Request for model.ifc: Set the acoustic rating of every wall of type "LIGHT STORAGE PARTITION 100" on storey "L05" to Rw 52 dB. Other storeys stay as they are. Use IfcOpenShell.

First a look at what the model holds.

```python
import ifcopenshell
import ifcopenshell.util.element

model = ifcopenshell.open("model.ifc")
print(model.schema)
storey = next(s for s in model.by_type("IfcBuildingStorey") if s.Name == "L05")
walls = [e for e in ifcopenshell.util.element.get_decomposition(storey) if e.is_a("IfcWall")]
seen = {}
for e in walls:
    element_type = ifcopenshell.util.element.get_type(e)
    key = (element_type.Name if element_type != e and element_type else None, ifcopenshell.util.element.get_pset(e, "Pset_WallCommon", "AcousticRating"))
    seen[key] = seen.get(key, 0) + 1
for (name, value), count in sorted(seen.items(), key=str):
    print(count, "x", name, "|", value)
```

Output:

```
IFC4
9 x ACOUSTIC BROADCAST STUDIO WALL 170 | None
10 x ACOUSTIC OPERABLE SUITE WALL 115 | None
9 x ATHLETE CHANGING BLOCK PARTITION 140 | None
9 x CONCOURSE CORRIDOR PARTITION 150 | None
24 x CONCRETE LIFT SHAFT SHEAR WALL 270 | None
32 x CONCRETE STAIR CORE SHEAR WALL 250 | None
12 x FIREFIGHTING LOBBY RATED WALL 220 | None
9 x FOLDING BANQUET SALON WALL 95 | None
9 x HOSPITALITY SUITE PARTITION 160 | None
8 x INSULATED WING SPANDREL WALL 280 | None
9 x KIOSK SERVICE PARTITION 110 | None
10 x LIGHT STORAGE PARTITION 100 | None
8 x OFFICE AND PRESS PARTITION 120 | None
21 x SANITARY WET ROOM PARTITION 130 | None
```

```python
import ifcopenshell
import ifcopenshell.api.pset
import ifcopenshell.util.element

model = ifcopenshell.open("model.ifc")

storey = next(s for s in model.by_type("IfcBuildingStorey") if s.Name == "L05")
walls = [e for e in ifcopenshell.util.element.get_decomposition(storey) if e.is_a("IfcWall")]

count = 0
for e in walls:
    element_type = ifcopenshell.util.element.get_type(e)
    if element_type in (None, e) or element_type.Name != "LIGHT STORAGE PARTITION 100":
        continue
    # add_pset returns the element's existing set when there is one.
    pset = ifcopenshell.api.pset.add_pset(model, product=e, name="Pset_WallCommon")
    ifcopenshell.api.pset.edit_pset(model, pset=pset, properties={"AcousticRating": "Rw 52 dB"})
    count += 1

print(count, "walls updated")

model.write("model_edited.ifc")
```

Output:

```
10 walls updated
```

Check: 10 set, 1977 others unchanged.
